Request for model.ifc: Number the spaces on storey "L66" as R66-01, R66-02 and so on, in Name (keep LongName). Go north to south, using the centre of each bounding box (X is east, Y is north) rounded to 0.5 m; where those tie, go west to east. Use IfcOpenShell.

First a look at what the model holds.

```python
import ifcopenshell
import ifcopenshell.util.element
import ifcopenshell.util.placement

model = ifcopenshell.open("model.ifc")
print(model.schema)
storey = next(s for s in model.by_type("IfcBuildingStorey") if s.Name == "L66")
spaces = [e for e in ifcopenshell.util.element.get_decomposition(storey) if e.is_a("IfcSpace")]
for e in sorted(spaces, key=lambda e: e.id()):
    origin = ifcopenshell.util.placement.get_local_placement(e.ObjectPlacement)[:3, 3]
    print(e.id(), e.Name, e.LongName, origin.round(2) + 0.0, sep=" | ")
```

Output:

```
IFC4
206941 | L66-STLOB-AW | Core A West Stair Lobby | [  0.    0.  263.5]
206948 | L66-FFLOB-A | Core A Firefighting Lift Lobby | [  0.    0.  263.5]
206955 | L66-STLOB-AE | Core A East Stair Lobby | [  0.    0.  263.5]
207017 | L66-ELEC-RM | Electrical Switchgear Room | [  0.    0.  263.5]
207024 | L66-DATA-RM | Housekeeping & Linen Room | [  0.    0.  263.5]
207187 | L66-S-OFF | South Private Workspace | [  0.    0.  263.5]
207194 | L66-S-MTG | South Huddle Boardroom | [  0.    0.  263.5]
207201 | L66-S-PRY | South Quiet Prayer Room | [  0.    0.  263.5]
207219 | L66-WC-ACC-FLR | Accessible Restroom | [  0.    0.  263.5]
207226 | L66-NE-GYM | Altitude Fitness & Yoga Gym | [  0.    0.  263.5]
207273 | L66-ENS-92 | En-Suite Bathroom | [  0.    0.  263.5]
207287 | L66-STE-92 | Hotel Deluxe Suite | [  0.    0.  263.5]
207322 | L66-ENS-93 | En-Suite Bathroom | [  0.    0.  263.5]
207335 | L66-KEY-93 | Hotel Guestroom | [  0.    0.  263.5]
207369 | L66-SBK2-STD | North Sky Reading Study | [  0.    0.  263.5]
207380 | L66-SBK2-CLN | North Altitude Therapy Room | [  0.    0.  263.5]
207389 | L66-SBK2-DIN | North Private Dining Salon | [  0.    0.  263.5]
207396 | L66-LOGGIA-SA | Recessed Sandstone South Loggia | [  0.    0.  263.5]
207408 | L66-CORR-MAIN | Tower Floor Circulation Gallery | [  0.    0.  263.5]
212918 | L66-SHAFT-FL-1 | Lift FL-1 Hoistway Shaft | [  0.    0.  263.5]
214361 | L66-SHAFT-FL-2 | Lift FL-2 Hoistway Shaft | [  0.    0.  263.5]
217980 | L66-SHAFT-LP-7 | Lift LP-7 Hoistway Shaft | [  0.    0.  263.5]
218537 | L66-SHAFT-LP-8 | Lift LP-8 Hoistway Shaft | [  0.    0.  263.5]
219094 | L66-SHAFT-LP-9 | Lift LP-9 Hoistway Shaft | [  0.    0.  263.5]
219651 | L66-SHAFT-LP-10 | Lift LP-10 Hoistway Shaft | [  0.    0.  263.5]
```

```python
import ifcopenshell
import ifcopenshell.geom
import ifcopenshell.util.element
import ifcopenshell.util.shape

model = ifcopenshell.open("model.ifc")
settings = ifcopenshell.geom.settings()
settings.set("use-world-coords", True)


def centre(element):
    shape = ifcopenshell.geom.create_shape(settings, element)
    return ifcopenshell.util.shape.get_bbox_centroid(shape.geometry)


storey = next(s for s in model.by_type("IfcBuildingStorey") if s.Name == "L66")
spaces = [e for e in ifcopenshell.util.element.get_decomposition(storey) if e.is_a("IfcSpace")]

# Insertion points can sit at a corner or the storey origin, so sort by the geometry (in metres).
centres = {e: centre(e) for e in spaces}
spaces.sort(key=lambda e: (-round(centres[e][1] / 0.5), centres[e][0]))

for i, e in enumerate(spaces, start=1):
    number = f"R66-{i:02d}"
    e.Name = number
    print(e.id(), number)

model.write("model_updated.ifc")
```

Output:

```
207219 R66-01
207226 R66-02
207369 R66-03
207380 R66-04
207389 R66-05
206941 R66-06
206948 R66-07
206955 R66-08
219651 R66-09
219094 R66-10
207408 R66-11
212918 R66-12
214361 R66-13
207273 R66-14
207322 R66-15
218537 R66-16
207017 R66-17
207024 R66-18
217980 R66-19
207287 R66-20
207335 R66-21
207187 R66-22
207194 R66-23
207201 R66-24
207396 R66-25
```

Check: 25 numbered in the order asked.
